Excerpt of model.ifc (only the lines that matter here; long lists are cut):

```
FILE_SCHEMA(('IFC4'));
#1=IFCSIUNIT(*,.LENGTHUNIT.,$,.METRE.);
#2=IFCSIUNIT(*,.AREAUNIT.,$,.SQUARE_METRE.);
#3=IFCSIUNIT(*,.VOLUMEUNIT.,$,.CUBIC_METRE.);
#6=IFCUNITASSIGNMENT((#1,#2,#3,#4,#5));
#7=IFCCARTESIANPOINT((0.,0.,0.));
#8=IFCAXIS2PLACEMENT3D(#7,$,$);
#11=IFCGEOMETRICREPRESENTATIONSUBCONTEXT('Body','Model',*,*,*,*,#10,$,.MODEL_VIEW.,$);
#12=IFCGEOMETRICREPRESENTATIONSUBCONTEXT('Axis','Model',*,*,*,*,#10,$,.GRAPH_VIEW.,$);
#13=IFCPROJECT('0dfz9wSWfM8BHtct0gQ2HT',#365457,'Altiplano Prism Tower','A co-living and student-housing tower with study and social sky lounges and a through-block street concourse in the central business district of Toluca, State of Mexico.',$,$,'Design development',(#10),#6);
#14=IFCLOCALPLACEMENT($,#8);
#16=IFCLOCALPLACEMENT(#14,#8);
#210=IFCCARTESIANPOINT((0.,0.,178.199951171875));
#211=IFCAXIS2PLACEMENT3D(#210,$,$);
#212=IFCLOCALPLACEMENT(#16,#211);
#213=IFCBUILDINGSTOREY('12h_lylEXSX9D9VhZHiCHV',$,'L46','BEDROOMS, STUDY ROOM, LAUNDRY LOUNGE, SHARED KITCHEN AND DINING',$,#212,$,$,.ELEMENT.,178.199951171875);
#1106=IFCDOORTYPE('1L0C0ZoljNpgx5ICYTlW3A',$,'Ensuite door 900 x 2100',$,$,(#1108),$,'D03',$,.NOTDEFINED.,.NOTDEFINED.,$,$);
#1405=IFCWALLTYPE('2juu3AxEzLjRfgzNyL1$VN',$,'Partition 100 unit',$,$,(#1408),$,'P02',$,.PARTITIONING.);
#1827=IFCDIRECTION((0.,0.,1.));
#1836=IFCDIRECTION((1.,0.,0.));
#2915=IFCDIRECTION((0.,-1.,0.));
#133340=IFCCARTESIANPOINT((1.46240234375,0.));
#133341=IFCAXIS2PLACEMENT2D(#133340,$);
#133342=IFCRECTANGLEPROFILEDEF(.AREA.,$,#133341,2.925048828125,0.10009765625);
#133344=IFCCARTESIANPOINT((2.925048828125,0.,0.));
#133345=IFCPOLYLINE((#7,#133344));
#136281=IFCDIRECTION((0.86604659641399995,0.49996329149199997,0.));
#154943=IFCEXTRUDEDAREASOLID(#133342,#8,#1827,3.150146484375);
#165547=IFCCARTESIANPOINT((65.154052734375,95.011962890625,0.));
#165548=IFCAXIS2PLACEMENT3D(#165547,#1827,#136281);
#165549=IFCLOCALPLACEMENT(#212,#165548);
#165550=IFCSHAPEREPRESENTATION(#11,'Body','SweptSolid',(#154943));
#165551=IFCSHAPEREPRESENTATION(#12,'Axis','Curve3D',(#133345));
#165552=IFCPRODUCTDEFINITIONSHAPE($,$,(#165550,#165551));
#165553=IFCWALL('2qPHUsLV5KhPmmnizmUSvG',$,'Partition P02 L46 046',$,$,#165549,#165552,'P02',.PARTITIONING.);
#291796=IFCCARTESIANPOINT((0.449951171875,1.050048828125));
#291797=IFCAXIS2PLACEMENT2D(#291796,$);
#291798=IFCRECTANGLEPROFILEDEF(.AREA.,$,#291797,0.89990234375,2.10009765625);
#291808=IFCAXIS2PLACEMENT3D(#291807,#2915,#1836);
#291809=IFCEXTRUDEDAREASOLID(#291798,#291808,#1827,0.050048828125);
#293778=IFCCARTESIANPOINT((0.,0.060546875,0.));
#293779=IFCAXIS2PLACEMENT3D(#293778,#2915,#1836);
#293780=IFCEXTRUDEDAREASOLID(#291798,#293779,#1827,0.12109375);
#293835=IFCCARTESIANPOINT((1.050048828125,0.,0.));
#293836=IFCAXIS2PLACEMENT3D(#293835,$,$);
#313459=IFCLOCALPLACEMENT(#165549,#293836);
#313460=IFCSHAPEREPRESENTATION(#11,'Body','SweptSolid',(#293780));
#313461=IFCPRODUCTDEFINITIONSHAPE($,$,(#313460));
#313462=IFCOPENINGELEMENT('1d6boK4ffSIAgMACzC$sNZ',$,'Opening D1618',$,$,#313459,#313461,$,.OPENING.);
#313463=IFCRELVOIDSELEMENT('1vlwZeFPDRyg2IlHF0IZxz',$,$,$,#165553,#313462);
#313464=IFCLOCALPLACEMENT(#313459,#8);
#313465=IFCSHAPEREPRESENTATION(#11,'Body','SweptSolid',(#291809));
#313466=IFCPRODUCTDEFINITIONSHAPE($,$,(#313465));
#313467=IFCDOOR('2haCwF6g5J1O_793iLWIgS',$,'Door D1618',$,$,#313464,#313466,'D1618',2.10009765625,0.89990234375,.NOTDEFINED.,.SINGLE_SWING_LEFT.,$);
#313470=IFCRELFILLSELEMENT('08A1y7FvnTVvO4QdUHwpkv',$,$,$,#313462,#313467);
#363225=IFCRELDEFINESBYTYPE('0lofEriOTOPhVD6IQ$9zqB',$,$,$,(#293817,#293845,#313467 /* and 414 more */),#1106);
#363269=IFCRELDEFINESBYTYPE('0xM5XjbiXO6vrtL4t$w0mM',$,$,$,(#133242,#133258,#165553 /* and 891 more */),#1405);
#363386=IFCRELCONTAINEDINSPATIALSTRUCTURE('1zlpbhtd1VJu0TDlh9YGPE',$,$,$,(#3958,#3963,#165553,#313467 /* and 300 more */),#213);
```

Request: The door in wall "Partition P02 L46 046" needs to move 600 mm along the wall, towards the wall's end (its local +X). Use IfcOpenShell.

```python
import ifcopenshell
import ifcopenshell.api.geometry
import ifcopenshell.util.placement

model = ifcopenshell.open("model.ifc")

door = model.by_id(313467)
opening = door.FillsVoids[0].RelatingOpeningElement
wall = opening.VoidsElements[0].RelatingBuildingElement

wall_matrix = ifcopenshell.util.placement.get_local_placement(wall.ObjectPlacement)
shift = wall_matrix[:3, 0] * 0.6
before = ifcopenshell.util.placement.get_local_placement(door.ObjectPlacement)[:3, 3].copy()

# The door is placed relative to its opening, so it follows when the opening moves.
matrix = ifcopenshell.util.placement.get_local_placement(opening.ObjectPlacement)
matrix[:3, 3] += shift
ifcopenshell.api.geometry.edit_object_placement(
    model, product=opening, matrix=matrix, is_si=False, should_transform_children=True
)

after = ifcopenshell.util.placement.get_local_placement(door.ObjectPlacement)[:3, 3]
print("door moved by", (after - before).round(3) + 0.0)

model.write("model_edited.ifc")
```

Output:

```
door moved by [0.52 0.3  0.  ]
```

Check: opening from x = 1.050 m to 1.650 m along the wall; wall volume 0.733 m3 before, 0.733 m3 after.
